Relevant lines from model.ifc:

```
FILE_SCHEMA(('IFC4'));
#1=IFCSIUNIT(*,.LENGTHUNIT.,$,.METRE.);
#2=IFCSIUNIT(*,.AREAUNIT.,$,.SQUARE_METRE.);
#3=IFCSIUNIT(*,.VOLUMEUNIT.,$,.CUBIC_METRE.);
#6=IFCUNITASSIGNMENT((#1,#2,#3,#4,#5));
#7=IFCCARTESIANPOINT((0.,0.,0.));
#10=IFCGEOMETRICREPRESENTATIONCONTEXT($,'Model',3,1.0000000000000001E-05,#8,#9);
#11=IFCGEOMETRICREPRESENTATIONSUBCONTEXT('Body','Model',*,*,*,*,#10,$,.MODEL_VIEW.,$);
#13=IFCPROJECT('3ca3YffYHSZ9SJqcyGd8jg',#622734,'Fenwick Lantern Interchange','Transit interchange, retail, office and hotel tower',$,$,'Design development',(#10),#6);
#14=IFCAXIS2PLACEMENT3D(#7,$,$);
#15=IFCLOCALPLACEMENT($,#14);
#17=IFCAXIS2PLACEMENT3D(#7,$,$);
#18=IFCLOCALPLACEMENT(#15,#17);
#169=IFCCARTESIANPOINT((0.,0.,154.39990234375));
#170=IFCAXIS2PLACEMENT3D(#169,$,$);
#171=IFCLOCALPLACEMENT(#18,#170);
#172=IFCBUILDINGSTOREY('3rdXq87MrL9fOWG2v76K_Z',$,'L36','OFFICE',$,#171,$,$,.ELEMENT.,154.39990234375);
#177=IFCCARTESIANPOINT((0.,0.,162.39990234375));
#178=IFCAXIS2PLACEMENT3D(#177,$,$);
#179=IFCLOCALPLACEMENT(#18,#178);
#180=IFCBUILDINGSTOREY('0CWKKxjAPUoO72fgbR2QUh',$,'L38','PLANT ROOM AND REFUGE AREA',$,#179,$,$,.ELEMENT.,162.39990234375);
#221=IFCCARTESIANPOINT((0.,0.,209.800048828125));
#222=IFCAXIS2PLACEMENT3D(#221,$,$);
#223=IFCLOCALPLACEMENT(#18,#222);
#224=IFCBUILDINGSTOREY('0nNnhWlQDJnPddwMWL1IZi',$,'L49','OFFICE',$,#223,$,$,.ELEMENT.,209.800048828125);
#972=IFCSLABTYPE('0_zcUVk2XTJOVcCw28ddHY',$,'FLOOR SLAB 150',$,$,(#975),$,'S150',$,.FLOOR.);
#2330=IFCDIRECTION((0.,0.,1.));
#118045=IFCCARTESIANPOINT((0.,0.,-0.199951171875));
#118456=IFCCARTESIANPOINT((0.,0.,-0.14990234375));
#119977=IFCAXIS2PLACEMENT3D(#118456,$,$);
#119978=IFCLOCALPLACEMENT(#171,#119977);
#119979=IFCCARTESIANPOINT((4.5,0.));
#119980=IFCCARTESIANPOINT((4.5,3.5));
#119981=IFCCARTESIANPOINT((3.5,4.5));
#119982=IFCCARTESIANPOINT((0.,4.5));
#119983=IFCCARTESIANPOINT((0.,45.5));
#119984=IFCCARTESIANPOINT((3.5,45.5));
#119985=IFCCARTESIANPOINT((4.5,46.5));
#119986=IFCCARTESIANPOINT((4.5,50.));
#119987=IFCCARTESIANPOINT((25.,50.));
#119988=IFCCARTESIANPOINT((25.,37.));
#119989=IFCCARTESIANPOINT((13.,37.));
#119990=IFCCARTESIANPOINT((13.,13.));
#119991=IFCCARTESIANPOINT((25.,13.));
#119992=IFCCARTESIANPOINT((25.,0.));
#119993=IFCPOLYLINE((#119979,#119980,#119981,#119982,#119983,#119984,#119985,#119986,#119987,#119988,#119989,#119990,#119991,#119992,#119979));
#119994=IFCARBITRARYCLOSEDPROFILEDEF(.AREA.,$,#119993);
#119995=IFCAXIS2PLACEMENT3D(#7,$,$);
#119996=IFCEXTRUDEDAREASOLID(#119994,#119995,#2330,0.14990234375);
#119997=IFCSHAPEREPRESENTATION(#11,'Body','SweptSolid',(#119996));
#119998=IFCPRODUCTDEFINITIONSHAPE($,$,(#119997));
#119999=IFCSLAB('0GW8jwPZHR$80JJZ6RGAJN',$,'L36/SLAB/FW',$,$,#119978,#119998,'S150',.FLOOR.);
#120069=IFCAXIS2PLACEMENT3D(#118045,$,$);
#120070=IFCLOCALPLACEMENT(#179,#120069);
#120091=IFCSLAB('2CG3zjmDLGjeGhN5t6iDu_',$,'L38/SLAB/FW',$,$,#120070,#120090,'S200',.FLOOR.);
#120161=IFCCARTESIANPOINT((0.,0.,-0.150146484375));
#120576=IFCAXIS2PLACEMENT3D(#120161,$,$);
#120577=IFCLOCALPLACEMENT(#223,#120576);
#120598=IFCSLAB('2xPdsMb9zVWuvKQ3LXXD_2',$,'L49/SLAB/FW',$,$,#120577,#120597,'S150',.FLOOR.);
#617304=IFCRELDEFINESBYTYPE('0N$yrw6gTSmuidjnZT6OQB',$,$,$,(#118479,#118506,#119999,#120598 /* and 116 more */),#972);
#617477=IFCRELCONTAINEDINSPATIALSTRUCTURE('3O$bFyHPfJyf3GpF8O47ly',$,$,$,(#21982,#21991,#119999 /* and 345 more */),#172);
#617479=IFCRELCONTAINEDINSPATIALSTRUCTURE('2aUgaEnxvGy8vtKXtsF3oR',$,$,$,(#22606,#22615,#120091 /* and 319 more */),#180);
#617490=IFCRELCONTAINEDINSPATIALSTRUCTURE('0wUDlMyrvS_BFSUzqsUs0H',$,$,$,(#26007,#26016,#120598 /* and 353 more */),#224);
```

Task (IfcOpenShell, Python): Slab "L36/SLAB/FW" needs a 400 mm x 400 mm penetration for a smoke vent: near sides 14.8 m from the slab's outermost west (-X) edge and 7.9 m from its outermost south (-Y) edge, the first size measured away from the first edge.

```python
import numpy as np
import ifcopenshell
import ifcopenshell.api.feature
import ifcopenshell.api.geometry
import ifcopenshell.api.root
import ifcopenshell.geom
import ifcopenshell.util.placement
import ifcopenshell.util.representation
import ifcopenshell.util.shape
import ifcopenshell.util.unit

model = ifcopenshell.open("model.ifc")
unit_scale = ifcopenshell.util.unit.calculate_unit_scale(model)
settings = ifcopenshell.geom.settings()


def volume(element):
    """Net volume in cubic metres, openings subtracted."""
    shape = ifcopenshell.geom.create_shape(settings, element)
    return ifcopenshell.util.shape.get_volume(shape.geometry)


slab = model.by_id(119999)
before = volume(slab)

# Extent in the slab's own axes, in metres. The edges named are its -X and -Y sides.
slab_shape = ifcopenshell.geom.create_shape(settings, slab)
vertices = ifcopenshell.util.shape.get_vertices(slab_shape.geometry)
x_min, y_min, bottom = vertices.min(axis=0)
top = vertices[:, 2].max()

opening = ifcopenshell.api.root.create_entity(model, ifc_class="IfcOpeningElement", name="Smoke vent opening", predefined_type="OPENING")
context = ifcopenshell.util.representation.get_context(model, "Model", "Body", "MODEL_VIEW")
width, depth = 0.4, 0.4
outline = [(0.0, 0.0), (width, 0.0), (width, depth), (0.0, depth), (0.0, 0.0)]
# Overshoot both faces by 50 mm so the cut is clean.
shape = ifcopenshell.api.geometry.add_slab_representation(
    model, context=context, depth=top - bottom + 0.1, polyline=outline
)
ifcopenshell.api.geometry.assign_representation(model, product=opening, representation=shape)

matrix = ifcopenshell.util.placement.get_local_placement(slab.ObjectPlacement)
matrix[:, 3] = matrix @ np.append(np.array([x_min + 14.8, y_min + 7.9, bottom - 0.05]) / unit_scale, 1.0)
ifcopenshell.api.geometry.edit_object_placement(model, product=opening, matrix=matrix, is_si=False)
ifcopenshell.api.feature.add_feature(model, feature=opening, element=slab)

after = volume(slab)

print(f"slab volume {before:.3f} -> {after:.3f} m3")

model.write("model_updated.ifc")
```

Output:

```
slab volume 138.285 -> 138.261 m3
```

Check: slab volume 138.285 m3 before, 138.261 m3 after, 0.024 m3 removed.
